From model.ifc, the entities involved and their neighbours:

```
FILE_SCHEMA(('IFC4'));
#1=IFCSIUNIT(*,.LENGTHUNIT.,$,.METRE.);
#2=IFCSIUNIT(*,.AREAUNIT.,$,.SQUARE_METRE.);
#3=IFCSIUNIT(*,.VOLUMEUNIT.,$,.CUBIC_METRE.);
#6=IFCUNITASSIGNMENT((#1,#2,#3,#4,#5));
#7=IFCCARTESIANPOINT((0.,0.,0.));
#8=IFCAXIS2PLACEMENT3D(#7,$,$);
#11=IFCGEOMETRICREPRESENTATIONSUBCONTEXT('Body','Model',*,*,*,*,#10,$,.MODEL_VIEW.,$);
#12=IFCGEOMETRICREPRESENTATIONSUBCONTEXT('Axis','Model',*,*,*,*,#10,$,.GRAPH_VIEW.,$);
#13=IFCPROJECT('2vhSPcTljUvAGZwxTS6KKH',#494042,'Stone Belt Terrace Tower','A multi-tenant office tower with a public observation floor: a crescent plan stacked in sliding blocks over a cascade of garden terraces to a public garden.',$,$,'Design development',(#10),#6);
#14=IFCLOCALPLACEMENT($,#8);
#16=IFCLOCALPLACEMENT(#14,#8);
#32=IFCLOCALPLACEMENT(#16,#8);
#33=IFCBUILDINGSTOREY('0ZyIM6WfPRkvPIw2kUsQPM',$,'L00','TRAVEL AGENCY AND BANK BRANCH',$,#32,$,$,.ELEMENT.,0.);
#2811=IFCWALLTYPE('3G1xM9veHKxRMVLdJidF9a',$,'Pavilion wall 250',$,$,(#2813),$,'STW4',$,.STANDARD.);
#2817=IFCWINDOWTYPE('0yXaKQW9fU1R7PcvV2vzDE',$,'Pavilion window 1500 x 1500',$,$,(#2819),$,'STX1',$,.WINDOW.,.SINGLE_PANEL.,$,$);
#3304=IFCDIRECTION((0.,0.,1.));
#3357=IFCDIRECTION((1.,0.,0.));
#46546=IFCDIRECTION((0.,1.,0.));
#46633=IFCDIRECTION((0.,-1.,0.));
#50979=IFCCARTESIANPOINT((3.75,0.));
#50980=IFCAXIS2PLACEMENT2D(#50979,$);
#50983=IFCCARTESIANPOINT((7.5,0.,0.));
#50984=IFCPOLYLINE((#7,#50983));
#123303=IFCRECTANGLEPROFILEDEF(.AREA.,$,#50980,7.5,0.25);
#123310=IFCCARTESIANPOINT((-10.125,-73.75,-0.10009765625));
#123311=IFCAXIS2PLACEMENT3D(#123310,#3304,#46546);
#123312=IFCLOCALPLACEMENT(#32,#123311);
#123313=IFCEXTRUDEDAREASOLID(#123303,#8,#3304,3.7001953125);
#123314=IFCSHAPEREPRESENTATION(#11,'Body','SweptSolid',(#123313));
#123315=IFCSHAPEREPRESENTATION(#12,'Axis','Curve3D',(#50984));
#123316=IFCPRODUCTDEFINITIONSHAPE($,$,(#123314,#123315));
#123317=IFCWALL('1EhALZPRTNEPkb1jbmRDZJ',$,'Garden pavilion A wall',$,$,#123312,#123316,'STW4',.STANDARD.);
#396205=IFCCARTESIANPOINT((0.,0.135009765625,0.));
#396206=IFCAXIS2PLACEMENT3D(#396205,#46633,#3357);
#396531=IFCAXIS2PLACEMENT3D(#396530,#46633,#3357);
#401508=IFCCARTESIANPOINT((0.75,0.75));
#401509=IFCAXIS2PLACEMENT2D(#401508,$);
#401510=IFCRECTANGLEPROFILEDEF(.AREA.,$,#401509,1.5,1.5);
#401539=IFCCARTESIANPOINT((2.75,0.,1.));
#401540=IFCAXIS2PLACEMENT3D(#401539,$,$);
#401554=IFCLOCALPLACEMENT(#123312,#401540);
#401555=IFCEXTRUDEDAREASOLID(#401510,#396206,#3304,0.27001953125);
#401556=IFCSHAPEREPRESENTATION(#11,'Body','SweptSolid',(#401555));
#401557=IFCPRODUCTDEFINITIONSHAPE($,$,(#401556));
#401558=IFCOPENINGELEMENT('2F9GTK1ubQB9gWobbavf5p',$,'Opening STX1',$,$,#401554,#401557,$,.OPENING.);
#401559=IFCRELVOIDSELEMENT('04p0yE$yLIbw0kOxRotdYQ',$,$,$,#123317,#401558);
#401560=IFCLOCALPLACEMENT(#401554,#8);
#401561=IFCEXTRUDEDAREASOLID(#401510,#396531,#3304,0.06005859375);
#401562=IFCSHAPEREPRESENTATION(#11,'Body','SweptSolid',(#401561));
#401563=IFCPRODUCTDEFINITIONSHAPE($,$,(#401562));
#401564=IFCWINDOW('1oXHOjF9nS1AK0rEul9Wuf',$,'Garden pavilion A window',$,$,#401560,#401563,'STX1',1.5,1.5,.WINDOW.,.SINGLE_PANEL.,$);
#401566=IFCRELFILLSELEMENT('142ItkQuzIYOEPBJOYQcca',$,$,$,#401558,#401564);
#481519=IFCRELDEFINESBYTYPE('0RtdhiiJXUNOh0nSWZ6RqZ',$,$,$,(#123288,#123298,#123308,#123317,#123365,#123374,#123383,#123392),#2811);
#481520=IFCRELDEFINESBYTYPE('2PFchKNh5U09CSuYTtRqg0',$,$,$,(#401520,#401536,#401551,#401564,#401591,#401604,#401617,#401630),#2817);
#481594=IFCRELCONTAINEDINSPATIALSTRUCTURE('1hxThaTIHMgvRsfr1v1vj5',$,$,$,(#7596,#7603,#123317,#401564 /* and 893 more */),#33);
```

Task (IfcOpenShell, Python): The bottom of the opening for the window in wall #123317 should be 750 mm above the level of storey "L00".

```python
import numpy as np
import ifcopenshell
import ifcopenshell.api.geometry
import ifcopenshell.geom
import ifcopenshell.util.element
import ifcopenshell.util.placement
import ifcopenshell.util.shape
import ifcopenshell.util.unit

model = ifcopenshell.open("model.ifc")
unit_scale = ifcopenshell.util.unit.calculate_unit_scale(model)

window = model.by_guid("1oXHOjF9nS1AK0rEul9Wuf")
opening = window.FillsVoids[0].RelatingOpeningElement
storey = ifcopenshell.util.element.get_container(window, ifc_class="IfcBuildingStorey")
level = ifcopenshell.util.placement.get_local_placement(storey.ObjectPlacement)[2, 3]

# The opening's origin need not be at the sill, so measure its lowest point.
shape = ifcopenshell.geom.create_shape(ifcopenshell.geom.settings(), opening)
bottom = ifcopenshell.util.shape.get_shape_bottom_elevation(shape, shape.geometry) / unit_scale
dz = level + 0.75 - bottom

shift = np.array([0.0, 0.0, dz])
# The window is placed relative to its opening, so it follows when the opening moves.
matrix = ifcopenshell.util.placement.get_local_placement(opening.ObjectPlacement)
matrix[:3, 3] += shift
ifcopenshell.api.geometry.edit_object_placement(
    model, product=opening, matrix=matrix, is_si=False, should_transform_children=True
)

print(f"moved by {dz * unit_scale:+.3f} m")

model.write("model_v2.ifc")
```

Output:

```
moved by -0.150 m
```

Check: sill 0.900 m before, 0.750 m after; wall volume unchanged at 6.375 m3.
